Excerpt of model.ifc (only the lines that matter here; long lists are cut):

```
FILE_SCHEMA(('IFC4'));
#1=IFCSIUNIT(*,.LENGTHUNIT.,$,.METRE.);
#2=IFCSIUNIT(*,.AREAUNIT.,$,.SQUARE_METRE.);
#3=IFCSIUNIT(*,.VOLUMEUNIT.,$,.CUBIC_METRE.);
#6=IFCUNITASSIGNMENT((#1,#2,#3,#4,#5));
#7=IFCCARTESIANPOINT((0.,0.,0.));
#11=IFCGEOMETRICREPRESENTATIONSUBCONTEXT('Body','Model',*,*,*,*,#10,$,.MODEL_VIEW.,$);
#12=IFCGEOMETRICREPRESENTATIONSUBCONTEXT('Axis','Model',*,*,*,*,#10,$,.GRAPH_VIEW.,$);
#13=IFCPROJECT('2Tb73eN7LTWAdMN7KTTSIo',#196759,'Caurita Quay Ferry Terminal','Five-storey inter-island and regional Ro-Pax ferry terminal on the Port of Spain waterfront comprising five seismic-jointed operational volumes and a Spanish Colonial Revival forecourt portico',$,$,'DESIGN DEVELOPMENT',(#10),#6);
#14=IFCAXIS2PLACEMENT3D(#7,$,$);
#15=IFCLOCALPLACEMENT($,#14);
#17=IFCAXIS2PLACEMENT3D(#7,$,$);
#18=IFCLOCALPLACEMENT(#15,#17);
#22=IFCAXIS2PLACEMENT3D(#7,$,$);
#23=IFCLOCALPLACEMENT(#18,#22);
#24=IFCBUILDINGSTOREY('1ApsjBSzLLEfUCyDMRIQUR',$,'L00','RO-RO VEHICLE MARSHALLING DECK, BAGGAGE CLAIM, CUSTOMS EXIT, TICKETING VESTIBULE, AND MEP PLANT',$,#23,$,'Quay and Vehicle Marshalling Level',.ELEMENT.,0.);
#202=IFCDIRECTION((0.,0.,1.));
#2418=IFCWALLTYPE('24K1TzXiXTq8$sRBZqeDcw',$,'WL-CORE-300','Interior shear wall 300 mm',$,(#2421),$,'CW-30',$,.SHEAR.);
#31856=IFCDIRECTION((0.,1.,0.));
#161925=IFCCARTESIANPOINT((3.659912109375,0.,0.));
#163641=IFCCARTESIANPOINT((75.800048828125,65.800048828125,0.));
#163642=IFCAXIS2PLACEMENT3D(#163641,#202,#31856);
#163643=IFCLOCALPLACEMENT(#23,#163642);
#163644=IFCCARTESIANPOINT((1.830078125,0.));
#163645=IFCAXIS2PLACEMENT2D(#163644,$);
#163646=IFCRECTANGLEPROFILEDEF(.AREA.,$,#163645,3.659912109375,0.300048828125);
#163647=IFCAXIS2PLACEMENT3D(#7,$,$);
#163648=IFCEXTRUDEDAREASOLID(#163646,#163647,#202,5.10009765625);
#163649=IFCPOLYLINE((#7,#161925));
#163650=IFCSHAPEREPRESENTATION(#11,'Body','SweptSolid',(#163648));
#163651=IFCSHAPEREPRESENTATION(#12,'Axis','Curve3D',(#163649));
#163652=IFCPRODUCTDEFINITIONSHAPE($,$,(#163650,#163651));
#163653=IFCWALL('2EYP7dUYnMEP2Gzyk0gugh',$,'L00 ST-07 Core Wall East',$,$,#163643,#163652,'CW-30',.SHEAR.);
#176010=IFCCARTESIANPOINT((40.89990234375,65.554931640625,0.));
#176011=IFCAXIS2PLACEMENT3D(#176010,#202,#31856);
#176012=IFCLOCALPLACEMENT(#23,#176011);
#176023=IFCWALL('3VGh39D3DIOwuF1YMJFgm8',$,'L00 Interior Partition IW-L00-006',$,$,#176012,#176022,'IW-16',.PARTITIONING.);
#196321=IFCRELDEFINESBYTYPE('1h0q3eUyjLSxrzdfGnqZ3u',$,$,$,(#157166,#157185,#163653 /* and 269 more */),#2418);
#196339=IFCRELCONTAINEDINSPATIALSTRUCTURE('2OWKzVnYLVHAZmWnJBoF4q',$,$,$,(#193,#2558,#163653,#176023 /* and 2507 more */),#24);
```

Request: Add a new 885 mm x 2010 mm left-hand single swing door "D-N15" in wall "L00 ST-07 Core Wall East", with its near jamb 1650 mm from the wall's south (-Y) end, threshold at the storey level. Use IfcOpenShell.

```python
import numpy as np
import ifcopenshell
import ifcopenshell.api.feature
import ifcopenshell.api.geometry
import ifcopenshell.api.root
import ifcopenshell.api.spatial
import ifcopenshell.geom
import ifcopenshell.util.element
import ifcopenshell.util.placement
import ifcopenshell.util.representation
import ifcopenshell.util.shape
import ifcopenshell.util.unit

model = ifcopenshell.open("model.ifc")
unit_scale = ifcopenshell.util.unit.calculate_unit_scale(model)
settings = ifcopenshell.geom.settings()


def volume(element):
    """Net volume in cubic metres, openings subtracted."""
    shape = ifcopenshell.geom.create_shape(settings, element)
    return ifcopenshell.util.shape.get_volume(shape.geometry)


wall = model.by_guid("2EYP7dUYnMEP2Gzyk0gugh")
storey = ifcopenshell.util.element.get_container(wall, ifc_class="IfcBuildingStorey")
context = ifcopenshell.util.representation.get_context(model, "Model", "Body", "MODEL_VIEW")
before = volume(wall)

width, height, from_end, sill = 0.885, 2.01, 1.65, 0.0  # metres

# The wall runs along its own X axis, and the end named is its -X end.
wall_shape = ifcopenshell.geom.create_shape(settings, wall)
x, y, z = ifcopenshell.util.shape.get_vertices(wall_shape.geometry).T
start = x.min() + from_end
face, thickness = float(y.min()), float(y.max() - y.min())
wall_matrix = ifcopenshell.util.placement.get_local_placement(wall.ObjectPlacement)
level = ifcopenshell.util.placement.get_local_placement(storey.ObjectPlacement)[2, 3]


def in_wall(x, y):
    """Placement at x, y metres in the wall's axes, at sill height."""
    matrix = wall_matrix.copy()
    matrix[:, 3] = wall_matrix @ np.array([x / unit_scale, y / unit_scale, 0.0, 1.0])
    matrix[2, 3] = level + sill / unit_scale
    return matrix


# Opening: a box that overshoots both wall faces by 50 mm.
opening = ifcopenshell.api.root.create_entity(model, ifc_class="IfcOpeningElement", predefined_type="OPENING")
box = ifcopenshell.api.geometry.add_wall_representation(
    model, context=context, length=width, height=height, thickness=thickness + 0.1
)
ifcopenshell.api.geometry.assign_representation(model, product=opening, representation=box)
ifcopenshell.api.geometry.edit_object_placement(model, product=opening, matrix=in_wall(start, face - 0.05), is_si=False)
ifcopenshell.api.feature.add_feature(model, feature=opening, element=wall)

door = ifcopenshell.api.root.create_entity(model, ifc_class="IfcDoor", name="D-N15", predefined_type="DOOR")
door.OverallWidth, door.OverallHeight = width / unit_scale, height / unit_scale
door.OperationType = "SINGLE_SWING_LEFT"
body = ifcopenshell.api.geometry.add_door_representation(
    model,
    context=context,
    overall_width=door.OverallWidth,
    overall_height=door.OverallHeight,
    operation_type="SINGLE_SWING_LEFT",
    lining_properties={"LiningDepth": thickness / unit_scale, "ThresholdDepth": thickness / unit_scale},
)
ifcopenshell.api.geometry.assign_representation(model, product=door, representation=body)
ifcopenshell.api.spatial.assign_container(model, products=[door], relating_structure=storey)
ifcopenshell.api.feature.add_filling(model, opening=opening, element=door)

# The lining spans the wall, so the door starts at the wall face.
ifcopenshell.api.geometry.edit_object_placement(model, product=door, matrix=in_wall(start, face), is_si=False)

after = volume(wall)

print(f"wall volume {before:.3f} -> {after:.3f} m3")

model.write("model_v2.ifc")
```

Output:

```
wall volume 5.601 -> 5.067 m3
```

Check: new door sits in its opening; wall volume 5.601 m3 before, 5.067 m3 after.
